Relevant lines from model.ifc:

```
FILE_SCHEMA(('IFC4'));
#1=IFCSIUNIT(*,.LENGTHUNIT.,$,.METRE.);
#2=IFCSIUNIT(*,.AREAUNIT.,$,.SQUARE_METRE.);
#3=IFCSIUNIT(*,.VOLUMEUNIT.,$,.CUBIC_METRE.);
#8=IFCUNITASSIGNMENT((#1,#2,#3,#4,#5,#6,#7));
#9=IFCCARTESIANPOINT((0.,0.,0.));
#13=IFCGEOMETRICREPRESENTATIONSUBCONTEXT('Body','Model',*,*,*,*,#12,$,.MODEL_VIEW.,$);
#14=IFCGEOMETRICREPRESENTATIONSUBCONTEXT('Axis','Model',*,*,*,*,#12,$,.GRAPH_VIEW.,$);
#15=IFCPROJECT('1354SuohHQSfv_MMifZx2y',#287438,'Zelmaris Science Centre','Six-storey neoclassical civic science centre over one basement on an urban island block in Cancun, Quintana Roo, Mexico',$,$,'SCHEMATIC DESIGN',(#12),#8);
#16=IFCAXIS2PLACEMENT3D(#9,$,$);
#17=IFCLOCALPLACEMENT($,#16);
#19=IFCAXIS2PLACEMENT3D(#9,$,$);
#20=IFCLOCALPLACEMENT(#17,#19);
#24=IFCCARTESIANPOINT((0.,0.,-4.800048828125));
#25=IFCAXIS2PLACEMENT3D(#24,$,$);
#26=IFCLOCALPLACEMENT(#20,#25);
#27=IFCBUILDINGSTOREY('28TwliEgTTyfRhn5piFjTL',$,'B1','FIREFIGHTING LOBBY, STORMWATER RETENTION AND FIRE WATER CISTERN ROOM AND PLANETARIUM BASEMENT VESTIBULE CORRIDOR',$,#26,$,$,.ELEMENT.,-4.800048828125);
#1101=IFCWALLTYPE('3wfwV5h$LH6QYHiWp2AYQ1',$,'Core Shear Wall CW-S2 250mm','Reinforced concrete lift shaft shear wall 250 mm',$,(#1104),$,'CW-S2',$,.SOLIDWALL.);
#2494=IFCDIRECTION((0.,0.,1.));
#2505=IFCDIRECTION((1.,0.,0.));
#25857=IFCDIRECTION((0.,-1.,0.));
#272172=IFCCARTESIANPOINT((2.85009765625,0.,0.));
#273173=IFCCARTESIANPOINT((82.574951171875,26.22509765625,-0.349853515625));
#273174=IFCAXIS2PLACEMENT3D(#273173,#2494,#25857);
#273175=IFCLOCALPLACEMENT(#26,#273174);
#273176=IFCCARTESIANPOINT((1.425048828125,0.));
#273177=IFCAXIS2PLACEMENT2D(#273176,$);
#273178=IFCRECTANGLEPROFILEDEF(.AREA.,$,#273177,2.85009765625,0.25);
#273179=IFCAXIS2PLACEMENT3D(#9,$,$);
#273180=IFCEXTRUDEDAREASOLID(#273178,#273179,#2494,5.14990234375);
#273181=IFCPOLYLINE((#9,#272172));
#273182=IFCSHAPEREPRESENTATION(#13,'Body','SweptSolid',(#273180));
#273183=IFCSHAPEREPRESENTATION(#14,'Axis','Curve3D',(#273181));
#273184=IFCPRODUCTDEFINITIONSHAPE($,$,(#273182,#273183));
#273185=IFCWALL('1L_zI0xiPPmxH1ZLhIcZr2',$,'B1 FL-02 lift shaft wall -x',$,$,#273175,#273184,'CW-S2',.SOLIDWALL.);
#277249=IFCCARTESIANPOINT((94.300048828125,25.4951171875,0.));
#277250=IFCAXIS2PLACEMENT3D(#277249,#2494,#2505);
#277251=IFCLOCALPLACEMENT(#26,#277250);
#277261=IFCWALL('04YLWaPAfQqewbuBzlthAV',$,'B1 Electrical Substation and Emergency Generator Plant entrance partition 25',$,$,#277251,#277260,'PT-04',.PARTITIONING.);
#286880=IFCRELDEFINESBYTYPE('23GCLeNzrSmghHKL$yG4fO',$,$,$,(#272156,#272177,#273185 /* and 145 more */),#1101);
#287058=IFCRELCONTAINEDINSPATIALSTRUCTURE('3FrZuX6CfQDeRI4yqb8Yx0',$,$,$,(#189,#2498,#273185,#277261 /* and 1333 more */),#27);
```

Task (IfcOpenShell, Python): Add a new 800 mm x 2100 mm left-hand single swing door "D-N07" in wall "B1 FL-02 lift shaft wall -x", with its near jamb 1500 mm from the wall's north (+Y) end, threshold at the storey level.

```python
import numpy as np
import ifcopenshell
import ifcopenshell.api.feature
import ifcopenshell.api.geometry
import ifcopenshell.api.root
import ifcopenshell.api.spatial
import ifcopenshell.geom
import ifcopenshell.util.element
import ifcopenshell.util.placement
import ifcopenshell.util.representation
import ifcopenshell.util.shape
import ifcopenshell.util.unit

model = ifcopenshell.open("model.ifc")
unit_scale = ifcopenshell.util.unit.calculate_unit_scale(model)
settings = ifcopenshell.geom.settings()


def volume(element):
    """Net volume in cubic metres, openings subtracted."""
    shape = ifcopenshell.geom.create_shape(settings, element)
    return ifcopenshell.util.shape.get_volume(shape.geometry)


wall = model.by_guid("1L_zI0xiPPmxH1ZLhIcZr2")
storey = ifcopenshell.util.element.get_container(wall, ifc_class="IfcBuildingStorey")
context = ifcopenshell.util.representation.get_context(model, "Model", "Body", "MODEL_VIEW")
before = volume(wall)

width, height, from_end, sill = 0.8, 2.1, 1.5, 0.0  # metres

# The wall runs along its own X axis, and the end named is its -X end.
wall_shape = ifcopenshell.geom.create_shape(settings, wall)
x, y, z = ifcopenshell.util.shape.get_vertices(wall_shape.geometry).T
start = x.min() + from_end
face, thickness = float(y.min()), float(y.max() - y.min())
wall_matrix = ifcopenshell.util.placement.get_local_placement(wall.ObjectPlacement)
level = ifcopenshell.util.placement.get_local_placement(storey.ObjectPlacement)[2, 3]


def in_wall(x, y):
    """Placement at x, y metres in the wall's axes, at sill height."""
    matrix = wall_matrix.copy()
    matrix[:, 3] = wall_matrix @ np.array([x / unit_scale, y / unit_scale, 0.0, 1.0])
    matrix[2, 3] = level + sill / unit_scale
    return matrix


# Opening: a box that overshoots both wall faces by 50 mm.
opening = ifcopenshell.api.root.create_entity(model, ifc_class="IfcOpeningElement", predefined_type="OPENING")
box = ifcopenshell.api.geometry.add_wall_representation(
    model, context=context, length=width, height=height, thickness=thickness + 0.1
)
ifcopenshell.api.geometry.assign_representation(model, product=opening, representation=box)
ifcopenshell.api.geometry.edit_object_placement(model, product=opening, matrix=in_wall(start, face - 0.05), is_si=False)
ifcopenshell.api.feature.add_feature(model, feature=opening, element=wall)

door = ifcopenshell.api.root.create_entity(model, ifc_class="IfcDoor", name="D-N07", predefined_type="DOOR")
door.OverallWidth, door.OverallHeight = width / unit_scale, height / unit_scale
door.OperationType = "SINGLE_SWING_LEFT"
body = ifcopenshell.api.geometry.add_door_representation(
    model,
    context=context,
    overall_width=door.OverallWidth,
    overall_height=door.OverallHeight,
    operation_type="SINGLE_SWING_LEFT",
    lining_properties={"LiningDepth": thickness / unit_scale, "ThresholdDepth": thickness / unit_scale},
)
ifcopenshell.api.geometry.assign_representation(model, product=door, representation=body)
ifcopenshell.api.spatial.assign_container(model, products=[door], relating_structure=storey)
ifcopenshell.api.feature.add_filling(model, opening=opening, element=door)

# The lining spans the wall, so the door starts at the wall face.
ifcopenshell.api.geometry.edit_object_placement(model, product=door, matrix=in_wall(start, face), is_si=False)

after = volume(wall)

print(f"wall volume {before:.3f} -> {after:.3f} m3")

model.write("model_rev.ifc")
```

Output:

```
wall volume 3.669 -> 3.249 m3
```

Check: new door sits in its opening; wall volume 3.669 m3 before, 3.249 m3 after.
